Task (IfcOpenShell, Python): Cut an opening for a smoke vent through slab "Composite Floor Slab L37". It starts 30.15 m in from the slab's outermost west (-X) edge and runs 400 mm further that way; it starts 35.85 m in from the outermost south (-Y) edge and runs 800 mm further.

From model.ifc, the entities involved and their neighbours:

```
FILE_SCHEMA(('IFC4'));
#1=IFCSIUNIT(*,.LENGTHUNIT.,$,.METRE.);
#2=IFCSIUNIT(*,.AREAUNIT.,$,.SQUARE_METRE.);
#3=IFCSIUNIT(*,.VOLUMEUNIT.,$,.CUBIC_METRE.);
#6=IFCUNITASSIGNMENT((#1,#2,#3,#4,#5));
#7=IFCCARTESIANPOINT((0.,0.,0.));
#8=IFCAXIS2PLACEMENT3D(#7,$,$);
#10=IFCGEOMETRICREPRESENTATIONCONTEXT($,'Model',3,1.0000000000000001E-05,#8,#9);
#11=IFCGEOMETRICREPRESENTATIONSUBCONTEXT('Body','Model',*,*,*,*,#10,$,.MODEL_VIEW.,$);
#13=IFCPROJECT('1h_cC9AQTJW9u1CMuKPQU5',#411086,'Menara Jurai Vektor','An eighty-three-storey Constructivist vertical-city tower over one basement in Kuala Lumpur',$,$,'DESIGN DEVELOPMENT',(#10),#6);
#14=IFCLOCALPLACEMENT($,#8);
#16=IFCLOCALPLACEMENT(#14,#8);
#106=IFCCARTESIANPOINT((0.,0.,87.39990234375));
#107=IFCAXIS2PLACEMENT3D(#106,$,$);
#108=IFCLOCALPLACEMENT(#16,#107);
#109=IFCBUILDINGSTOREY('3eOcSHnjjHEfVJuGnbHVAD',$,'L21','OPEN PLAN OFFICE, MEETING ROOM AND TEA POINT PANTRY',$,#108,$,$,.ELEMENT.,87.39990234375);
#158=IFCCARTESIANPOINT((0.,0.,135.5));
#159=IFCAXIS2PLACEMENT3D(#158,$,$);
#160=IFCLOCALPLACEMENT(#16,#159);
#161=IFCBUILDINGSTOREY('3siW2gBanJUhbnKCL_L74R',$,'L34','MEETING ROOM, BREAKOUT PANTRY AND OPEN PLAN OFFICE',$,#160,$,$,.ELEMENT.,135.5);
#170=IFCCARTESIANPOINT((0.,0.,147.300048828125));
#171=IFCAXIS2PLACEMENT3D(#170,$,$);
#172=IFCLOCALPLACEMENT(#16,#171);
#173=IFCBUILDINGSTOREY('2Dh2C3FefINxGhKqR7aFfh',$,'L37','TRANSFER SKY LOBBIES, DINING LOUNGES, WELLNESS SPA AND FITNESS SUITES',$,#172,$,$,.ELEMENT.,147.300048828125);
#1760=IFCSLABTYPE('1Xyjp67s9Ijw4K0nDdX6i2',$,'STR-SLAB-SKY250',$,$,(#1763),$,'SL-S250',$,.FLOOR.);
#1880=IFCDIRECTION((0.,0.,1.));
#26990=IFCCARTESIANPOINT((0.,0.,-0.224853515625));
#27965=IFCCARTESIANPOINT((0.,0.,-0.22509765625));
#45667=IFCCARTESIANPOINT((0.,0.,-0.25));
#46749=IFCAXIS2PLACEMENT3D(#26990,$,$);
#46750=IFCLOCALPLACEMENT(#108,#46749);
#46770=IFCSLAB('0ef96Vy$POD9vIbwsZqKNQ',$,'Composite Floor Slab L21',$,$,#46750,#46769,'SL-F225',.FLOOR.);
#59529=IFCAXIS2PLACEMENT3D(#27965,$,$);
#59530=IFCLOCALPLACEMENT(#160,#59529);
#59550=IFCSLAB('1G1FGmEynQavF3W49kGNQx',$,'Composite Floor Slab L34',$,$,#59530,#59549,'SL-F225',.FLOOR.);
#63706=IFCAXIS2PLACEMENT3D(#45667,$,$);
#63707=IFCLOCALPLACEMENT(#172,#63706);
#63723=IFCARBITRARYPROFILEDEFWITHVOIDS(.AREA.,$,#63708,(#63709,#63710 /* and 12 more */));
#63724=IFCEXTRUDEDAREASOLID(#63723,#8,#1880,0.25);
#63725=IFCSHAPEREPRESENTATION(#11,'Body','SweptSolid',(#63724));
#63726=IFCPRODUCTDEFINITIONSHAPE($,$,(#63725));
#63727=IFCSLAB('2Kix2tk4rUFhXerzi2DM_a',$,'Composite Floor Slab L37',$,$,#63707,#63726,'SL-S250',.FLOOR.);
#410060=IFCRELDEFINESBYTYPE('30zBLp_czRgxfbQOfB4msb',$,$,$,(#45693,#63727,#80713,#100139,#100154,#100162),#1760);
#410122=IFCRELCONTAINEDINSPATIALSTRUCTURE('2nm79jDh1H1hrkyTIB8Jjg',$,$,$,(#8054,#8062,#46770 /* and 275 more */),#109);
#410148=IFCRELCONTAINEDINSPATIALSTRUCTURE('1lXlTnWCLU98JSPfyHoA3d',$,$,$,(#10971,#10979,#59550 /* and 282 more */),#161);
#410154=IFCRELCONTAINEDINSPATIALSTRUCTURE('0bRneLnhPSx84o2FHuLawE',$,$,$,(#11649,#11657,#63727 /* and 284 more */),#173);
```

```python
import numpy as np
import ifcopenshell
import ifcopenshell.api.feature
import ifcopenshell.api.geometry
import ifcopenshell.api.root
import ifcopenshell.geom
import ifcopenshell.util.placement
import ifcopenshell.util.representation
import ifcopenshell.util.shape
import ifcopenshell.util.unit

model = ifcopenshell.open("model.ifc")
unit_scale = ifcopenshell.util.unit.calculate_unit_scale(model)
settings = ifcopenshell.geom.settings()


def volume(element):
    """Net volume in cubic metres, openings subtracted."""
    shape = ifcopenshell.geom.create_shape(settings, element)
    return ifcopenshell.util.shape.get_volume(shape.geometry)


slab = model.by_id(63727)
before = volume(slab)

# Extent in the slab's own axes, in metres. The edges named are its -X and -Y sides.
slab_shape = ifcopenshell.geom.create_shape(settings, slab)
vertices = ifcopenshell.util.shape.get_vertices(slab_shape.geometry)
x_min, y_min, bottom = vertices.min(axis=0)
top = vertices[:, 2].max()

opening = ifcopenshell.api.root.create_entity(model, ifc_class="IfcOpeningElement", name="Smoke vent opening", predefined_type="OPENING")
context = ifcopenshell.util.representation.get_context(model, "Model", "Body", "MODEL_VIEW")
width, depth = 0.4, 0.8
outline = [(0.0, 0.0), (width, 0.0), (width, depth), (0.0, depth), (0.0, 0.0)]
# Overshoot both faces by 50 mm so the cut is clean.
shape = ifcopenshell.api.geometry.add_slab_representation(
    model, context=context, depth=top - bottom + 0.1, polyline=outline
)
ifcopenshell.api.geometry.assign_representation(model, product=opening, representation=shape)

matrix = ifcopenshell.util.placement.get_local_placement(slab.ObjectPlacement)
matrix[:, 3] = matrix @ np.append(np.array([x_min + 30.15, y_min + 35.85, bottom - 0.05]) / unit_scale, 1.0)
ifcopenshell.api.geometry.edit_object_placement(model, product=opening, matrix=matrix, is_si=False)
ifcopenshell.api.feature.add_feature(model, feature=opening, element=slab)

after = volume(slab)

print(f"slab volume {before:.3f} -> {after:.3f} m3")

model.write("model-out.ifc")
```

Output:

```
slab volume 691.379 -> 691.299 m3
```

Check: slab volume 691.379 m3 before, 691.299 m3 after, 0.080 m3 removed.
